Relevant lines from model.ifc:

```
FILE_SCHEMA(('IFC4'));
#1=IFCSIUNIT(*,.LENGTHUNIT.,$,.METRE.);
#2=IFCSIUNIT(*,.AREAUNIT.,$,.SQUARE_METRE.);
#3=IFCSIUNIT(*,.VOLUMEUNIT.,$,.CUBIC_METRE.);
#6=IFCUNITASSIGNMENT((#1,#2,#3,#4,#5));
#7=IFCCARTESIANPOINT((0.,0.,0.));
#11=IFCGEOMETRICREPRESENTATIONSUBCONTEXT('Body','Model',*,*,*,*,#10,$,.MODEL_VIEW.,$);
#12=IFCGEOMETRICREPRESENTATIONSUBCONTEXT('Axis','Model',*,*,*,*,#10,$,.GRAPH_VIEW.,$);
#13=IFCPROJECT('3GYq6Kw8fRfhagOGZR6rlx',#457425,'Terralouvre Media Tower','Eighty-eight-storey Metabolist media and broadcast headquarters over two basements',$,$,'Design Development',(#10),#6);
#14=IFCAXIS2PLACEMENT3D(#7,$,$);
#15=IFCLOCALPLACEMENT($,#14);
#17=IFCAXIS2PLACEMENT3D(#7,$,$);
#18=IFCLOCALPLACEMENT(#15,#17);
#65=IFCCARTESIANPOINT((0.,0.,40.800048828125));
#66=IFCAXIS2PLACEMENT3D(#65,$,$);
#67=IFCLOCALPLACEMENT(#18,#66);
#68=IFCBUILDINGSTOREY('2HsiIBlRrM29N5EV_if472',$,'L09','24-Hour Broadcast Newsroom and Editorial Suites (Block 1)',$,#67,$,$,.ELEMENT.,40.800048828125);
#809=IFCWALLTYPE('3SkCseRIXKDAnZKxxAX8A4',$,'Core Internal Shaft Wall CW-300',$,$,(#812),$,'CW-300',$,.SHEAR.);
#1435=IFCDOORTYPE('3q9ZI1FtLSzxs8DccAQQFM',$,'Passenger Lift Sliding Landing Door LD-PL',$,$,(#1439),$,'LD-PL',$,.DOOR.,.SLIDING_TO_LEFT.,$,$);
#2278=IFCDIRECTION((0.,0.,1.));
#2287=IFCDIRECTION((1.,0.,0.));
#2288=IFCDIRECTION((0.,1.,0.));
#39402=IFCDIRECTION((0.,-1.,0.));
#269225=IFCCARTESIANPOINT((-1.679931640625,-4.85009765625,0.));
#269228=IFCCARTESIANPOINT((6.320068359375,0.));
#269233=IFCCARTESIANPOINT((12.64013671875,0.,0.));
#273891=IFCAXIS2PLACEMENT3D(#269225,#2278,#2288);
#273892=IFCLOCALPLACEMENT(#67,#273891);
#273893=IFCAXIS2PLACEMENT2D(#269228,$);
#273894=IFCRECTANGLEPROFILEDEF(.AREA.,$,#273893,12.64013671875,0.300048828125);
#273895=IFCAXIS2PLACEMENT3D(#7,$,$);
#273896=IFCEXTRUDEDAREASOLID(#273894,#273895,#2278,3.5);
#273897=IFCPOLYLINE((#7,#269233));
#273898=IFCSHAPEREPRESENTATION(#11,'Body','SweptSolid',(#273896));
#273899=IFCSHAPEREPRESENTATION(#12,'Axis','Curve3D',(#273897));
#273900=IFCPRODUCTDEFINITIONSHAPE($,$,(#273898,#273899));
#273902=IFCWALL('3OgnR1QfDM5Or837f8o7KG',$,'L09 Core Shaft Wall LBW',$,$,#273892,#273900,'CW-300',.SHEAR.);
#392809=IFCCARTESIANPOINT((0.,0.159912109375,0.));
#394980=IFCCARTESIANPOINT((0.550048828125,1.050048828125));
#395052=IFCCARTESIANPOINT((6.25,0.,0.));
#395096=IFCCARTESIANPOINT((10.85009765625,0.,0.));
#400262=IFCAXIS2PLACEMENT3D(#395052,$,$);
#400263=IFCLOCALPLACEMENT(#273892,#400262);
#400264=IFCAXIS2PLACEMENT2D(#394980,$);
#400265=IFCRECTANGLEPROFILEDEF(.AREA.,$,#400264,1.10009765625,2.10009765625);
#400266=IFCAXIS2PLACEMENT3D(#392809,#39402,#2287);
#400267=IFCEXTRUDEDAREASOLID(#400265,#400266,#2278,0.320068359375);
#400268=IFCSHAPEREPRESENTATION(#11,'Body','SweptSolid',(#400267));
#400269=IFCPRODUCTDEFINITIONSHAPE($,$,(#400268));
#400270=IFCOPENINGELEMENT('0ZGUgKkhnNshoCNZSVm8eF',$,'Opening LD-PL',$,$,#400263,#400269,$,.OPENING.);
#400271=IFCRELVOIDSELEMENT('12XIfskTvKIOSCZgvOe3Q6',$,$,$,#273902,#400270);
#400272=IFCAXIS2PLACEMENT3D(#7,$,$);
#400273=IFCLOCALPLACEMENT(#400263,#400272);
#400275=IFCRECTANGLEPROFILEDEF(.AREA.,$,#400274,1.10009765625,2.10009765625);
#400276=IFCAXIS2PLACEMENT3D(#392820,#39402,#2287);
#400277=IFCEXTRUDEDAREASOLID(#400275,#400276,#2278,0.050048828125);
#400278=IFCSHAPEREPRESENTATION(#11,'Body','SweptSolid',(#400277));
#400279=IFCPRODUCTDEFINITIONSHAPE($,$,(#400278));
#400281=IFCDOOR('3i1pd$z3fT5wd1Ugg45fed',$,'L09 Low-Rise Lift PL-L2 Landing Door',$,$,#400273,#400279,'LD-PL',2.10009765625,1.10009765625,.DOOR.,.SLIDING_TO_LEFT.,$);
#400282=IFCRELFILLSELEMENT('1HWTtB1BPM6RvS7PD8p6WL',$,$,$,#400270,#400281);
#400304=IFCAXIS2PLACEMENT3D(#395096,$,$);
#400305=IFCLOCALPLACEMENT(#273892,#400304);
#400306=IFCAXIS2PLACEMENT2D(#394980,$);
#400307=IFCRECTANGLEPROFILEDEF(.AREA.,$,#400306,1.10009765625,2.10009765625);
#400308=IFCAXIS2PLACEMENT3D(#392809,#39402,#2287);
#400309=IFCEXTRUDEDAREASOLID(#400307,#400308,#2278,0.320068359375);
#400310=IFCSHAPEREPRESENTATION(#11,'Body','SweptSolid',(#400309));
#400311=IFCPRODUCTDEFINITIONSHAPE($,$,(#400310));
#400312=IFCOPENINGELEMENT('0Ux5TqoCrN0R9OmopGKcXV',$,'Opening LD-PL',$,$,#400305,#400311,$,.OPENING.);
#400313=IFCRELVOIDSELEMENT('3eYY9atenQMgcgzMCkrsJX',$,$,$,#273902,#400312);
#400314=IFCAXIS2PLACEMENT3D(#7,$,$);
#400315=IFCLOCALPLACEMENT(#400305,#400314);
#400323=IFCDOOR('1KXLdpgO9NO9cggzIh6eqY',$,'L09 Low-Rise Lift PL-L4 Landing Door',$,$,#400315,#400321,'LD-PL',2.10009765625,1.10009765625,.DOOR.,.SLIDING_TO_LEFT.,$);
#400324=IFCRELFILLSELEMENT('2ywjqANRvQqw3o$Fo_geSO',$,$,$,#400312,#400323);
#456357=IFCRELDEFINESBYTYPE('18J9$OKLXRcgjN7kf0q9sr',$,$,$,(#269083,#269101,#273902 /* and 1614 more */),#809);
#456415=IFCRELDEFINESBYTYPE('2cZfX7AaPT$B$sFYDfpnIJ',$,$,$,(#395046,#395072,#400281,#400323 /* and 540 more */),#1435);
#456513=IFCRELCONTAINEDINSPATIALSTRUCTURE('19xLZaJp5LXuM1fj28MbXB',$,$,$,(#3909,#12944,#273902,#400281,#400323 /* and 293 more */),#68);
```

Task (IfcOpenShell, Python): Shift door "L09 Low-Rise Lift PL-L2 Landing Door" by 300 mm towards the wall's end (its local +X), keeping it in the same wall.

```python
import ifcopenshell
import ifcopenshell.api.geometry
import ifcopenshell.util.placement
import ifcopenshell.util.unit

model = ifcopenshell.open("model.ifc")
unit_scale = ifcopenshell.util.unit.calculate_unit_scale(model)

door = model.by_guid("3i1pd$z3fT5wd1Ugg45fed")
opening = door.FillsVoids[0].RelatingOpeningElement
wall = opening.VoidsElements[0].RelatingBuildingElement

wall_matrix = ifcopenshell.util.placement.get_local_placement(wall.ObjectPlacement)
shift = wall_matrix[:3, 0] * 0.3 / unit_scale
before = ifcopenshell.util.placement.get_local_placement(door.ObjectPlacement)[:3, 3].copy()

# The door is placed relative to its opening, so it follows when the opening moves.
matrix = ifcopenshell.util.placement.get_local_placement(opening.ObjectPlacement)
matrix[:3, 3] += shift
ifcopenshell.api.geometry.edit_object_placement(
    model, product=opening, matrix=matrix, is_si=False, should_transform_children=True
)

after = ifcopenshell.util.placement.get_local_placement(door.ObjectPlacement)[:3, 3]
print("door moved by", (after - before).round(3) + 0.0)

model.write("model_edited.ifc")
```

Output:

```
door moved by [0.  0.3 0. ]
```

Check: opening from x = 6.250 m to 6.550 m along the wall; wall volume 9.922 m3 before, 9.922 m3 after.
